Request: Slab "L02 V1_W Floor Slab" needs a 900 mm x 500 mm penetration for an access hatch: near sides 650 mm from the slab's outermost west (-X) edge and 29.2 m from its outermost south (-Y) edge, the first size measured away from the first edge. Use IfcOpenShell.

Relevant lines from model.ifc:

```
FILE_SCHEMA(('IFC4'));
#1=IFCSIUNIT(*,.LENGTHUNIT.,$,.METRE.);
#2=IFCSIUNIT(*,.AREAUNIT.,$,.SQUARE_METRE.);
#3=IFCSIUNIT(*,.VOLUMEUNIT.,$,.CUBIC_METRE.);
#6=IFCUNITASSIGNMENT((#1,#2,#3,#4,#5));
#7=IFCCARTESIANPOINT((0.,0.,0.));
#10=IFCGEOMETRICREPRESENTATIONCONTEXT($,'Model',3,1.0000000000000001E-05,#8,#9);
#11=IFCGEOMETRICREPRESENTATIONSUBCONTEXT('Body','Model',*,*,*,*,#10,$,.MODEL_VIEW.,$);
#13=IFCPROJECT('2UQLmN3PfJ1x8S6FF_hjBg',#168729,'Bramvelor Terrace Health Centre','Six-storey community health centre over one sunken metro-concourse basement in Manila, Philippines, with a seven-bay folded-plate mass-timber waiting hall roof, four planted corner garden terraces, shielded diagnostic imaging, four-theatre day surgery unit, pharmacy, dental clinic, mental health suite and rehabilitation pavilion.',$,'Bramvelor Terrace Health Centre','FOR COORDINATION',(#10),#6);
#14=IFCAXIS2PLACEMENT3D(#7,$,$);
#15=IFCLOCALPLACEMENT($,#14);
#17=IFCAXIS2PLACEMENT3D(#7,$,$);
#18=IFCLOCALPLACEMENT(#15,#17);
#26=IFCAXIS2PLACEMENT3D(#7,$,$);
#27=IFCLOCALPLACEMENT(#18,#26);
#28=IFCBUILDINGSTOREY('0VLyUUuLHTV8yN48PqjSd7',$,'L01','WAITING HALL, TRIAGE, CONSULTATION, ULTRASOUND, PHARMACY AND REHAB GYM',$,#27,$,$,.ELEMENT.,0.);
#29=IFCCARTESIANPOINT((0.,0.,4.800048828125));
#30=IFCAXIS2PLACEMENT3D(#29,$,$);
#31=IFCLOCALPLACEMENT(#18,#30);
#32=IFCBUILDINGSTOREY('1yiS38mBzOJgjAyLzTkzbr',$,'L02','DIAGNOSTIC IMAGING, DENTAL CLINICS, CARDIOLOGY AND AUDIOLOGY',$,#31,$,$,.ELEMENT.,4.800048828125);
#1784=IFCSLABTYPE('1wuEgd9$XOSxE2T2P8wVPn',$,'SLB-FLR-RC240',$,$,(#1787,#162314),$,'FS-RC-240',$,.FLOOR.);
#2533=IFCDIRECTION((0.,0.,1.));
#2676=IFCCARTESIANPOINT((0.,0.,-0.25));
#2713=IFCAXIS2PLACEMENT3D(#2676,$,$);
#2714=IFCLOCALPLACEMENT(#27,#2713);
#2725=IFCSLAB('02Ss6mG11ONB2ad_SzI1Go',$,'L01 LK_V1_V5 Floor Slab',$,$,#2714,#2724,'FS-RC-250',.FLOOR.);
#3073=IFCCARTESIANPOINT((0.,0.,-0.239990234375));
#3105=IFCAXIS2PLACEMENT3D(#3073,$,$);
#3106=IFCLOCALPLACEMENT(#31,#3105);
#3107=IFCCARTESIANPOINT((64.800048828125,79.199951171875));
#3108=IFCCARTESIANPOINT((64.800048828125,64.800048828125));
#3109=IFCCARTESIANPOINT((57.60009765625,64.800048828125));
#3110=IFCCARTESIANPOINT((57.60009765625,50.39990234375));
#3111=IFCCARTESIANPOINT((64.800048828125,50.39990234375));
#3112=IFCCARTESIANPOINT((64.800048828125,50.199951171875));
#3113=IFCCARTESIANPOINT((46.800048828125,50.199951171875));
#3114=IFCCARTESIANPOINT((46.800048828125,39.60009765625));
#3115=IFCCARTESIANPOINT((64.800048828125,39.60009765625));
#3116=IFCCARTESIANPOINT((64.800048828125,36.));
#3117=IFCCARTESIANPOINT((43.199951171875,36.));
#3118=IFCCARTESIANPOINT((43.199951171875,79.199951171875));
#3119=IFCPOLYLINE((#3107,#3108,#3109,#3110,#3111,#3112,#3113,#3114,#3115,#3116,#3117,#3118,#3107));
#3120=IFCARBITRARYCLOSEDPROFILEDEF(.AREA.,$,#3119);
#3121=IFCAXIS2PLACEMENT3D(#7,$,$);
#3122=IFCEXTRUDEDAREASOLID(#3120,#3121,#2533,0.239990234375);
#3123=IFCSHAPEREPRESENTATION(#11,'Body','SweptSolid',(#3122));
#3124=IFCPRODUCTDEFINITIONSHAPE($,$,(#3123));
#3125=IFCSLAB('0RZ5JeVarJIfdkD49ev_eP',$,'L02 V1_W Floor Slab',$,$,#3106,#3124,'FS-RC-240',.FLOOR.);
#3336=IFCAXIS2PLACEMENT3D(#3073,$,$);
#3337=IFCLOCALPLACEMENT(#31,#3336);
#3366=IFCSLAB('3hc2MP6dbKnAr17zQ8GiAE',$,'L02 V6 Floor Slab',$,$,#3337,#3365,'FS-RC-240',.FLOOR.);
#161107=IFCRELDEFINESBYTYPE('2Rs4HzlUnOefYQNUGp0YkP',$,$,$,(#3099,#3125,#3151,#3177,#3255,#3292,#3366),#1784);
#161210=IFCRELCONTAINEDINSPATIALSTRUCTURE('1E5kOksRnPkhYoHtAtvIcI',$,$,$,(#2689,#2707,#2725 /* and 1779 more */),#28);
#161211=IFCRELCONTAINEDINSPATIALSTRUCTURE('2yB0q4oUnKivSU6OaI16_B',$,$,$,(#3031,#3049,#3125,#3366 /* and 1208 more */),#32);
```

```python
import numpy as np
import ifcopenshell
import ifcopenshell.api.feature
import ifcopenshell.api.geometry
import ifcopenshell.api.root
import ifcopenshell.geom
import ifcopenshell.util.placement
import ifcopenshell.util.representation
import ifcopenshell.util.shape
import ifcopenshell.util.unit

model = ifcopenshell.open("model.ifc")
unit_scale = ifcopenshell.util.unit.calculate_unit_scale(model)
settings = ifcopenshell.geom.settings()


def volume(element):
    """Net volume in cubic metres, openings subtracted."""
    shape = ifcopenshell.geom.create_shape(settings, element)
    return ifcopenshell.util.shape.get_volume(shape.geometry)


slab = model.by_guid("0RZ5JeVarJIfdkD49ev_eP")
before = volume(slab)

# Extent in the slab's own axes, in metres. The edges named are its -X and -Y sides.
slab_shape = ifcopenshell.geom.create_shape(settings, slab)
vertices = ifcopenshell.util.shape.get_vertices(slab_shape.geometry)
x_min, y_min, bottom = vertices.min(axis=0)
top = vertices[:, 2].max()

opening = ifcopenshell.api.root.create_entity(model, ifc_class="IfcOpeningElement", name="Access hatch opening", predefined_type="OPENING")
context = ifcopenshell.util.representation.get_context(model, "Model", "Body", "MODEL_VIEW")
width, depth = 0.9, 0.5
outline = [(0.0, 0.0), (width, 0.0), (width, depth), (0.0, depth), (0.0, 0.0)]
# Overshoot both faces by 50 mm so the cut is clean.
shape = ifcopenshell.api.geometry.add_slab_representation(
    model, context=context, depth=top - bottom + 0.1, polyline=outline
)
ifcopenshell.api.geometry.assign_representation(model, product=opening, representation=shape)

matrix = ifcopenshell.util.placement.get_local_placement(slab.ObjectPlacement)
matrix[:, 3] = matrix @ np.append(np.array([x_min + 0.65, y_min + 29.2, bottom - 0.05]) / unit_scale, 1.0)
ifcopenshell.api.geometry.edit_object_placement(model, product=opening, matrix=matrix, is_si=False)
ifcopenshell.api.feature.add_feature(model, feature=opening, element=slab)

after = volume(slab)

print(f"slab volume {before:.3f} -> {after:.3f} m3")

model.write("model_edited.ifc")
```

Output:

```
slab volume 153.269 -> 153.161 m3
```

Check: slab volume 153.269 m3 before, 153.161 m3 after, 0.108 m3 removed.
